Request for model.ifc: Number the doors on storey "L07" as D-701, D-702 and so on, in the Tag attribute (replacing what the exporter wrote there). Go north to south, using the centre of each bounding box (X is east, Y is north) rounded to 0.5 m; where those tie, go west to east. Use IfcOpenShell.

First a look at what the model holds.

```python
import ifcopenshell
import ifcopenshell.util.element
import ifcopenshell.util.placement

model = ifcopenshell.open("model.ifc")
print(model.schema)
storey = next(s for s in model.by_type("IfcBuildingStorey") if s.Name == "L07")
doors = [e for e in ifcopenshell.util.element.get_decomposition(storey) if e.is_a("IfcDoor")]
for e in sorted(doors, key=lambda e: e.id()):
    origin = ifcopenshell.util.placement.get_local_placement(e.ObjectPlacement)[:3, 3]
    print(e.id(), e.Tag, e.Name, origin.round(2) + 0.0, sep=" | ")
```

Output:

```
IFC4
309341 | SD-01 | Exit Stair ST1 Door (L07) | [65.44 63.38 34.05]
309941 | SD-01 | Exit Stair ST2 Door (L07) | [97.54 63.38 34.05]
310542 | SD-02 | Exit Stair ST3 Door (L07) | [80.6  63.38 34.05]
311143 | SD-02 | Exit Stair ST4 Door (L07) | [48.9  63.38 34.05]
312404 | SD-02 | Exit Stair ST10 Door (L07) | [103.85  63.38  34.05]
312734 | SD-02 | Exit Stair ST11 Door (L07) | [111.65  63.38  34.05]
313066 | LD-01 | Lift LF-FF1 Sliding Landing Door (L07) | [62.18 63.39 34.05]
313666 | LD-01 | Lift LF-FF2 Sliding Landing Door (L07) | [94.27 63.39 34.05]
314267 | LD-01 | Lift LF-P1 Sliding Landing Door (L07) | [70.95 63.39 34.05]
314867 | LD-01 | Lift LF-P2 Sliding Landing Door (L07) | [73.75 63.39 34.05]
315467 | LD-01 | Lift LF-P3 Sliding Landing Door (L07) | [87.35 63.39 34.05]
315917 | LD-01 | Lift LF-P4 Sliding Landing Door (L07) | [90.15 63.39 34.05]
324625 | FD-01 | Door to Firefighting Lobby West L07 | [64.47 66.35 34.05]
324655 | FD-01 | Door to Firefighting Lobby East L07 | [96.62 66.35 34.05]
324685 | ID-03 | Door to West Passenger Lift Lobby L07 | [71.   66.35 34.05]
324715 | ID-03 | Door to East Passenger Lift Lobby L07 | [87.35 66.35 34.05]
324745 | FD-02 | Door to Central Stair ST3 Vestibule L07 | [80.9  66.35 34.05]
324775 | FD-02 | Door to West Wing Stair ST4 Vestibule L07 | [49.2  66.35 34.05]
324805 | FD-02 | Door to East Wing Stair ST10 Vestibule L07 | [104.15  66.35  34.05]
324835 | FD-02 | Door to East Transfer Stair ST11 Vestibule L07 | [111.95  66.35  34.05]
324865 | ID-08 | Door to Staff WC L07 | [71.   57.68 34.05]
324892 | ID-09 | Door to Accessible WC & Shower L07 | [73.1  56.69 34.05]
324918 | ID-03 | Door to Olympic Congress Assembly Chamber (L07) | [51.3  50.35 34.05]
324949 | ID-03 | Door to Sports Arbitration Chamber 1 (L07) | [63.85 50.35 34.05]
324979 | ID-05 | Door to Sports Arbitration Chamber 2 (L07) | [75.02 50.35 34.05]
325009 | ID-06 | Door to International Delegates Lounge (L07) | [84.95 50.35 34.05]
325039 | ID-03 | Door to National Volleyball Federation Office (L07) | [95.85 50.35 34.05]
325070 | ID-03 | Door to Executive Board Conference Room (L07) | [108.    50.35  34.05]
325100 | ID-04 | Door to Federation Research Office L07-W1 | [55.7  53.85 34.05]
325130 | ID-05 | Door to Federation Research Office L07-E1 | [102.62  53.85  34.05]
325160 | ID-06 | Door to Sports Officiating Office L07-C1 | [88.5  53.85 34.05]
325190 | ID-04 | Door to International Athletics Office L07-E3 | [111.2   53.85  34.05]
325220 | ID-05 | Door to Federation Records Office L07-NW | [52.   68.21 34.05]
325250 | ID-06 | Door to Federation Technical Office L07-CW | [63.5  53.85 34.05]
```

```python
import ifcopenshell
import ifcopenshell.geom
import ifcopenshell.util.element
import ifcopenshell.util.shape

model = ifcopenshell.open("model.ifc")
settings = ifcopenshell.geom.settings()
settings.set("use-world-coords", True)


def centre(element):
    shape = ifcopenshell.geom.create_shape(settings, element)
    return ifcopenshell.util.shape.get_bbox_centroid(shape.geometry)


storey = next(s for s in model.by_type("IfcBuildingStorey") if s.Name == "L07")
doors = [e for e in ifcopenshell.util.element.get_decomposition(storey) if e.is_a("IfcDoor")]

# Insertion points can sit at a corner or the storey origin, so sort by the geometry (in metres).
centres = {e: centre(e) for e in doors}
doors.sort(key=lambda e: (-round(centres[e][1] / 0.5), centres[e][0]))

for i, e in enumerate(doors, start=1):
    number = f"D-7{i:02d}"
    e.Tag = number
    print(e.id(), number)

model.write("model_edited.ifc")
```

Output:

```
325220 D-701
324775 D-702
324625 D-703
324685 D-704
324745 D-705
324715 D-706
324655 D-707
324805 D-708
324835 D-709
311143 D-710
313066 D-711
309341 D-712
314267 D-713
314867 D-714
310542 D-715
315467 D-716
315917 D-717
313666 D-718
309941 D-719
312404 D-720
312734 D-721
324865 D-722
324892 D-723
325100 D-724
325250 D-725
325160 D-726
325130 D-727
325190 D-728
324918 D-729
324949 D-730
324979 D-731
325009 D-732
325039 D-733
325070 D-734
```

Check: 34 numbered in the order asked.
